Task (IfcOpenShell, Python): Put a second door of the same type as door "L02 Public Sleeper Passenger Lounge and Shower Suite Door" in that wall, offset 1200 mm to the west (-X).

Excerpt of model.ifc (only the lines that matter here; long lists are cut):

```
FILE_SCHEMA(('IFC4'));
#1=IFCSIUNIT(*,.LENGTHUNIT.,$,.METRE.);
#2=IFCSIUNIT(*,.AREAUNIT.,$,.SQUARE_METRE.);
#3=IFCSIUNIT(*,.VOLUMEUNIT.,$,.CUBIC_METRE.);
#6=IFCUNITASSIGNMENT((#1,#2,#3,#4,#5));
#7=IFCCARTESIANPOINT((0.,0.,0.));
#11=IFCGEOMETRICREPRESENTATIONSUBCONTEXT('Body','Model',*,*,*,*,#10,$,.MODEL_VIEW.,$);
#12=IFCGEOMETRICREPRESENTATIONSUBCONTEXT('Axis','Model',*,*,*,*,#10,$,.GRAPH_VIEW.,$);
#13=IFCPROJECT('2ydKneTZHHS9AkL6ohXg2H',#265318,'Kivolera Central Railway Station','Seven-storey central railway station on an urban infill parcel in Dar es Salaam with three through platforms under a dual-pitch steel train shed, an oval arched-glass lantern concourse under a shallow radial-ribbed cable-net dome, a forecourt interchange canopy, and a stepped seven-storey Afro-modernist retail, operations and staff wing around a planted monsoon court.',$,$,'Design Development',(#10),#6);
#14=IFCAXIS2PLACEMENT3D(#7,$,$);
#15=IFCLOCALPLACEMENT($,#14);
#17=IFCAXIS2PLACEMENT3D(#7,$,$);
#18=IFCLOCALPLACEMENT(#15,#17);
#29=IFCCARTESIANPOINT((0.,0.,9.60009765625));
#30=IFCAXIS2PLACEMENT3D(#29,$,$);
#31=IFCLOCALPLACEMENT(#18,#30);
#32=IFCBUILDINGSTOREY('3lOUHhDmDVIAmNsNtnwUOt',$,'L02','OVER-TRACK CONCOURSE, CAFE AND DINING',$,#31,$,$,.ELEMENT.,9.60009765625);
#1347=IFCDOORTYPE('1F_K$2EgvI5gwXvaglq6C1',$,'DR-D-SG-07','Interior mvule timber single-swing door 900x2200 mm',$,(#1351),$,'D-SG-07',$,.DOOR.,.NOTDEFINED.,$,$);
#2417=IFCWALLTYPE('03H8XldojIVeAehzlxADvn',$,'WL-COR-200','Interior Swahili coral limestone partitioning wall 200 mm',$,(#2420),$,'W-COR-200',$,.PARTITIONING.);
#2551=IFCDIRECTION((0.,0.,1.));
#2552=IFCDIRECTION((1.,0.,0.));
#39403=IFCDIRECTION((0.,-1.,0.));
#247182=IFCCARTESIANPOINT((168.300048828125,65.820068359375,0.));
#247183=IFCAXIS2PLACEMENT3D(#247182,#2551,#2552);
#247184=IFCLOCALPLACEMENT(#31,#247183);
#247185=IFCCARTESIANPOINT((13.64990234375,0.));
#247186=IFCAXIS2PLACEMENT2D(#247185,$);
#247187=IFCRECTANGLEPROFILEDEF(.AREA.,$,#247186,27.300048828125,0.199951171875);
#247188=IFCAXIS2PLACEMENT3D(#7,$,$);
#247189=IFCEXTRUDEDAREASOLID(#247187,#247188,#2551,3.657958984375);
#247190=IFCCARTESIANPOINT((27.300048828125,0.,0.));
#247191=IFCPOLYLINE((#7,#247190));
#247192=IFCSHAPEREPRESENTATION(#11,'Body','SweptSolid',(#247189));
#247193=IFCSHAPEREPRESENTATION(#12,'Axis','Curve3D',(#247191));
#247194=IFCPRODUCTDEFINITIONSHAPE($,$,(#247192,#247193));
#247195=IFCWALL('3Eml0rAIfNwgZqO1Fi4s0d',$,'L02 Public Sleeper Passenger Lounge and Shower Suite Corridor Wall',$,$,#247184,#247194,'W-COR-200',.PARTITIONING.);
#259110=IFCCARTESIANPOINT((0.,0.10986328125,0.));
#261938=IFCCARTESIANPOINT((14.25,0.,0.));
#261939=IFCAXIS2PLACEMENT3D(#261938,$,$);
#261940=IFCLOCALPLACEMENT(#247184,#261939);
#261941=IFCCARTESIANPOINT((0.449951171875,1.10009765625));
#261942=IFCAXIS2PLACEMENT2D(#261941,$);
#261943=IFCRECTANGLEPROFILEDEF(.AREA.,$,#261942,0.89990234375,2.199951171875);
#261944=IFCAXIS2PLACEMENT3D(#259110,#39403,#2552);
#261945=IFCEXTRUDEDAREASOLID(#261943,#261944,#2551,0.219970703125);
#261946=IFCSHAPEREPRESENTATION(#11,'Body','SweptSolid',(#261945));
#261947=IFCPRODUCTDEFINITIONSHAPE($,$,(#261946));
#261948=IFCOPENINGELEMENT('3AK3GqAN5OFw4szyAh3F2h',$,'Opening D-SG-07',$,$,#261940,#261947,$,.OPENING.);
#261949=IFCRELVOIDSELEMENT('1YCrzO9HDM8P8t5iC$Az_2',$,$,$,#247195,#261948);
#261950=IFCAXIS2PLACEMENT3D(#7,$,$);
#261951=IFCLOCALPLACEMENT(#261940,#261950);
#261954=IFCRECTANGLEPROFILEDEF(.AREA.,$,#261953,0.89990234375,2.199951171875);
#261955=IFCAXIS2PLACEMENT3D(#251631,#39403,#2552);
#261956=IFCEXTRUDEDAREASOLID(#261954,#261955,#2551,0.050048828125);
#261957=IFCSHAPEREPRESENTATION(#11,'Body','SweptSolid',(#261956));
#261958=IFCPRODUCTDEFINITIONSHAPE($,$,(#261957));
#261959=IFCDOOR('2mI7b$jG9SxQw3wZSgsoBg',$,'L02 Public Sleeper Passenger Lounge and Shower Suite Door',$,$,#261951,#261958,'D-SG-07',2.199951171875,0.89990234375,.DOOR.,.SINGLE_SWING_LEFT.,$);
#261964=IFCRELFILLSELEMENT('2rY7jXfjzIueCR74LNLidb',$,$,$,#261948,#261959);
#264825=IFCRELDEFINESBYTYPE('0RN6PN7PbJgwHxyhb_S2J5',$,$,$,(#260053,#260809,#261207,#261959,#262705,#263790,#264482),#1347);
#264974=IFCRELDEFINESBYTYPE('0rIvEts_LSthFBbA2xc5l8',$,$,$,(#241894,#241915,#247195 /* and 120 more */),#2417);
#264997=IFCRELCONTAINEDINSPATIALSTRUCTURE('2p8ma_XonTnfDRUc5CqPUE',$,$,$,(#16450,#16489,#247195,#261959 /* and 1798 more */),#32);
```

```python
import ifcopenshell
import ifcopenshell.api.feature
import ifcopenshell.api.geometry
import ifcopenshell.api.root
import ifcopenshell.geom
import ifcopenshell.util.element
import ifcopenshell.util.placement
import ifcopenshell.util.shape
import ifcopenshell.util.unit

model = ifcopenshell.open("model.ifc")
unit_scale = ifcopenshell.util.unit.calculate_unit_scale(model)
settings = ifcopenshell.geom.settings()


def volume(element):
    """Net volume in cubic metres, openings subtracted."""
    shape = ifcopenshell.geom.create_shape(settings, element)
    return ifcopenshell.util.shape.get_volume(shape.geometry)


door = model.by_id(261959)
opening = door.FillsVoids[0].RelatingOpeningElement
wall = opening.VoidsElements[0].RelatingBuildingElement
before = volume(wall)
shift = ifcopenshell.util.placement.get_local_placement(wall.ObjectPlacement)[:3, 0] * -1.2 / unit_scale

# copy_class copies the void relationship, type, container and properties, but no geometry.
new_opening = ifcopenshell.api.root.copy_class(model, product=opening)
new_opening.Representation = ifcopenshell.util.element.copy_deep(
    model, opening.Representation, exclude=["IfcGeometricRepresentationContext", "IfcRepresentationMap"]
)
new_door = ifcopenshell.api.root.copy_class(model, product=door)
new_door.Representation = ifcopenshell.util.element.copy_deep(
    model, door.Representation, exclude=["IfcGeometricRepresentationContext", "IfcRepresentationMap"]
)
new_door.Tag = None
ifcopenshell.api.feature.add_filling(model, opening=new_opening, element=new_door)

for old, new in ((opening, new_opening), (door, new_door)):
    matrix = ifcopenshell.util.placement.get_local_placement(old.ObjectPlacement)
    matrix[:3, 3] += shift
    ifcopenshell.api.geometry.edit_object_placement(model, product=new, matrix=matrix, is_si=False)

after = volume(wall)

print(f"wall volume {before:.3f} -> {after:.3f} m3")

model.write("model_updated.ifc")
```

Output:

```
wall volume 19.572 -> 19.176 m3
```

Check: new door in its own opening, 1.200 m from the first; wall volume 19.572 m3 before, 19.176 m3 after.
